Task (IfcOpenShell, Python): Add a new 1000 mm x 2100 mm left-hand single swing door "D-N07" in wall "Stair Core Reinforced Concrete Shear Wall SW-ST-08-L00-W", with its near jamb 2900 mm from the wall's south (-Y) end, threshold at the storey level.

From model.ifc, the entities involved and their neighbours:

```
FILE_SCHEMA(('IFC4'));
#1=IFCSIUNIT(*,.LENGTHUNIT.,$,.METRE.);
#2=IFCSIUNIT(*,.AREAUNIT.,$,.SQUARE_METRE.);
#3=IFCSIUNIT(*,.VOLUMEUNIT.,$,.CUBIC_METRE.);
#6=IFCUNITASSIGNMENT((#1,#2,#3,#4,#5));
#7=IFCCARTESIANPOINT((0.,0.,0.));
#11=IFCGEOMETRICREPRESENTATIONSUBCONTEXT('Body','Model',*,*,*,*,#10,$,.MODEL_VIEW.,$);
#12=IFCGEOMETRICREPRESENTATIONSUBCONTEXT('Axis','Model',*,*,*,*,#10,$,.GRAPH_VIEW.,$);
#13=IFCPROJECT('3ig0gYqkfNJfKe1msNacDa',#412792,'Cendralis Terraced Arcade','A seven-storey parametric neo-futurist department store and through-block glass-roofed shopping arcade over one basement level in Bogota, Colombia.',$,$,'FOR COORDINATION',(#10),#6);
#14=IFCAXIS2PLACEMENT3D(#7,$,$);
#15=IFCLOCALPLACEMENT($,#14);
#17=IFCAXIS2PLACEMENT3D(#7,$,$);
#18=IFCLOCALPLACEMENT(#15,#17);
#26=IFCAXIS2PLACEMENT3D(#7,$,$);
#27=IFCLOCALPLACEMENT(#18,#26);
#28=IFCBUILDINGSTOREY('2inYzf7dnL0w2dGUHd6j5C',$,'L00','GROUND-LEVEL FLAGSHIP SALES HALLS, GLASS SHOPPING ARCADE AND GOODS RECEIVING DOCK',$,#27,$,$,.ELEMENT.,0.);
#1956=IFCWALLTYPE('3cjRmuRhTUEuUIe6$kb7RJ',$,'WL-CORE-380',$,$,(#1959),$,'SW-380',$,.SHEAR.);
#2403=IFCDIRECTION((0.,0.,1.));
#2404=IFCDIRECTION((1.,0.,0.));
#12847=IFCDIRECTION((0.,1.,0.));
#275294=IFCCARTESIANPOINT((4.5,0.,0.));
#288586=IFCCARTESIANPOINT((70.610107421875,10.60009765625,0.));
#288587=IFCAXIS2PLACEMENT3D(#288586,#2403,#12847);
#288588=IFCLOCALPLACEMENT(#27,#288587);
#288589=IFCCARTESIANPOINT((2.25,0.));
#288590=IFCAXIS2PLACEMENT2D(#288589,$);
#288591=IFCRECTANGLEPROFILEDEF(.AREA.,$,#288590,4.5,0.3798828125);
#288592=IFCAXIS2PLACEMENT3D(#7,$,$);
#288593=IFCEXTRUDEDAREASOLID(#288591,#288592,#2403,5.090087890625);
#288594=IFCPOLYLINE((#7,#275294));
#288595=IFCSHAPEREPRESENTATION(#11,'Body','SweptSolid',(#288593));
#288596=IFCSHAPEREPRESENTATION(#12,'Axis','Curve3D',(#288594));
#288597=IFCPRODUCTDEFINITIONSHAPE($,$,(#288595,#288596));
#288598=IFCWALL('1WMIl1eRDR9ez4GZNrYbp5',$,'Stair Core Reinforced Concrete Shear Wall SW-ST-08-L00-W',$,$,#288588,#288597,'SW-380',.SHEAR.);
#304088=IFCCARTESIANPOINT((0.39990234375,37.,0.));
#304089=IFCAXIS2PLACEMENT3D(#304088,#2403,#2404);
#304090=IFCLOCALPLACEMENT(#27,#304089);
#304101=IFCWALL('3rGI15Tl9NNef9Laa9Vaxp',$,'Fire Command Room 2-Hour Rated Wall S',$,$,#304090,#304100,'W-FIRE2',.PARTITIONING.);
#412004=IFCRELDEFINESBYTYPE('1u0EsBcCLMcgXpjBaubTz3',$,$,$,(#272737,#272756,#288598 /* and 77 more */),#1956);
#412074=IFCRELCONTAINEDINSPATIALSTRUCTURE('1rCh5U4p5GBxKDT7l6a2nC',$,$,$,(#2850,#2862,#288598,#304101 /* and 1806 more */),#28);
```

```python
import numpy as np
import ifcopenshell
import ifcopenshell.api.feature
import ifcopenshell.api.geometry
import ifcopenshell.api.root
import ifcopenshell.api.spatial
import ifcopenshell.geom
import ifcopenshell.util.element
import ifcopenshell.util.placement
import ifcopenshell.util.representation
import ifcopenshell.util.shape
import ifcopenshell.util.unit

model = ifcopenshell.open("model.ifc")
unit_scale = ifcopenshell.util.unit.calculate_unit_scale(model)
settings = ifcopenshell.geom.settings()


def volume(element):
    """Net volume in cubic metres, openings subtracted."""
    shape = ifcopenshell.geom.create_shape(settings, element)
    return ifcopenshell.util.shape.get_volume(shape.geometry)


wall = model.by_guid("1WMIl1eRDR9ez4GZNrYbp5")
storey = ifcopenshell.util.element.get_container(wall, ifc_class="IfcBuildingStorey")
context = ifcopenshell.util.representation.get_context(model, "Model", "Body", "MODEL_VIEW")
before = volume(wall)

width, height, from_end, sill = 1, 2.1, 2.9, 0.0  # metres

# The wall runs along its own X axis, and the end named is its -X end.
wall_shape = ifcopenshell.geom.create_shape(settings, wall)
x, y, z = ifcopenshell.util.shape.get_vertices(wall_shape.geometry).T
start = x.min() + from_end
face, thickness = float(y.min()), float(y.max() - y.min())
wall_matrix = ifcopenshell.util.placement.get_local_placement(wall.ObjectPlacement)
level = ifcopenshell.util.placement.get_local_placement(storey.ObjectPlacement)[2, 3]


def in_wall(x, y):
    """Placement at x, y metres in the wall's axes, at sill height."""
    matrix = wall_matrix.copy()
    matrix[:, 3] = wall_matrix @ np.array([x / unit_scale, y / unit_scale, 0.0, 1.0])
    matrix[2, 3] = level + sill / unit_scale
    return matrix


# Opening: a box that overshoots both wall faces by 50 mm.
opening = ifcopenshell.api.root.create_entity(model, ifc_class="IfcOpeningElement", predefined_type="OPENING")
box = ifcopenshell.api.geometry.add_wall_representation(
    model, context=context, length=width, height=height, thickness=thickness + 0.1
)
ifcopenshell.api.geometry.assign_representation(model, product=opening, representation=box)
ifcopenshell.api.geometry.edit_object_placement(model, product=opening, matrix=in_wall(start, face - 0.05), is_si=False)
ifcopenshell.api.feature.add_feature(model, feature=opening, element=wall)

door = ifcopenshell.api.root.create_entity(model, ifc_class="IfcDoor", name="D-N07", predefined_type="DOOR")
door.OverallWidth, door.OverallHeight = width / unit_scale, height / unit_scale
door.OperationType = "SINGLE_SWING_LEFT"
body = ifcopenshell.api.geometry.add_door_representation(
    model,
    context=context,
    overall_width=door.OverallWidth,
    overall_height=door.OverallHeight,
    operation_type="SINGLE_SWING_LEFT",
    lining_properties={"LiningDepth": thickness / unit_scale, "ThresholdDepth": thickness / unit_scale},
)
ifcopenshell.api.geometry.assign_representation(model, product=door, representation=body)
ifcopenshell.api.spatial.assign_container(model, products=[door], relating_structure=storey)
ifcopenshell.api.feature.add_filling(model, opening=opening, element=door)

# The lining spans the wall, so the door starts at the wall face.
ifcopenshell.api.geometry.edit_object_placement(model, product=door, matrix=in_wall(start, face), is_si=False)

after = volume(wall)

print(f"wall volume {before:.3f} -> {after:.3f} m3")

model.write("model-out.ifc")
```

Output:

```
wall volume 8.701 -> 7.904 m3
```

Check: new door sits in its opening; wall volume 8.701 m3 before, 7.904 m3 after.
